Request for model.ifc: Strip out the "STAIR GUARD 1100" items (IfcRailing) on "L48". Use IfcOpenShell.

First a look at what the model holds.

```python
import ifcopenshell
import ifcopenshell.util.element

model = ifcopenshell.open("model.ifc")
print(model.schema)
storey = next(s for s in model.by_type("IfcBuildingStorey") if s.Name == "L48")
railings = [e for e in ifcopenshell.util.element.get_decomposition(storey) if e.is_a("IfcRailing")]
seen = {}
for e in railings:
    element_type = ifcopenshell.util.element.get_type(e)
    name = element_type.Name if element_type not in (None, e) else None
    seen[name] = seen.get(name, 0) + 1
for name, count in sorted(seen.items(), key=str):
    print(count, "x", name)
```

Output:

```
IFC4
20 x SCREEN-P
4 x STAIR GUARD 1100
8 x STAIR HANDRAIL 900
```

```python
import ifcopenshell
import ifcopenshell.api.root
import ifcopenshell.util.element

model = ifcopenshell.open("model.ifc")

storey = next(s for s in model.by_type("IfcBuildingStorey") if s.Name == "L48")
railings = [e for e in ifcopenshell.util.element.get_decomposition(storey) if e.is_a("IfcRailing")]
targets = [e for e in railings if (t := ifcopenshell.util.element.get_type(e)) not in (None, e) and t.Name == "STAIR GUARD 1100"]

for e in targets:
    ifcopenshell.api.root.remove_product(model, product=e)
print(len(targets), "removed")

model.write("model_updated.ifc")
```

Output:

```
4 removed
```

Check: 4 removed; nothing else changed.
